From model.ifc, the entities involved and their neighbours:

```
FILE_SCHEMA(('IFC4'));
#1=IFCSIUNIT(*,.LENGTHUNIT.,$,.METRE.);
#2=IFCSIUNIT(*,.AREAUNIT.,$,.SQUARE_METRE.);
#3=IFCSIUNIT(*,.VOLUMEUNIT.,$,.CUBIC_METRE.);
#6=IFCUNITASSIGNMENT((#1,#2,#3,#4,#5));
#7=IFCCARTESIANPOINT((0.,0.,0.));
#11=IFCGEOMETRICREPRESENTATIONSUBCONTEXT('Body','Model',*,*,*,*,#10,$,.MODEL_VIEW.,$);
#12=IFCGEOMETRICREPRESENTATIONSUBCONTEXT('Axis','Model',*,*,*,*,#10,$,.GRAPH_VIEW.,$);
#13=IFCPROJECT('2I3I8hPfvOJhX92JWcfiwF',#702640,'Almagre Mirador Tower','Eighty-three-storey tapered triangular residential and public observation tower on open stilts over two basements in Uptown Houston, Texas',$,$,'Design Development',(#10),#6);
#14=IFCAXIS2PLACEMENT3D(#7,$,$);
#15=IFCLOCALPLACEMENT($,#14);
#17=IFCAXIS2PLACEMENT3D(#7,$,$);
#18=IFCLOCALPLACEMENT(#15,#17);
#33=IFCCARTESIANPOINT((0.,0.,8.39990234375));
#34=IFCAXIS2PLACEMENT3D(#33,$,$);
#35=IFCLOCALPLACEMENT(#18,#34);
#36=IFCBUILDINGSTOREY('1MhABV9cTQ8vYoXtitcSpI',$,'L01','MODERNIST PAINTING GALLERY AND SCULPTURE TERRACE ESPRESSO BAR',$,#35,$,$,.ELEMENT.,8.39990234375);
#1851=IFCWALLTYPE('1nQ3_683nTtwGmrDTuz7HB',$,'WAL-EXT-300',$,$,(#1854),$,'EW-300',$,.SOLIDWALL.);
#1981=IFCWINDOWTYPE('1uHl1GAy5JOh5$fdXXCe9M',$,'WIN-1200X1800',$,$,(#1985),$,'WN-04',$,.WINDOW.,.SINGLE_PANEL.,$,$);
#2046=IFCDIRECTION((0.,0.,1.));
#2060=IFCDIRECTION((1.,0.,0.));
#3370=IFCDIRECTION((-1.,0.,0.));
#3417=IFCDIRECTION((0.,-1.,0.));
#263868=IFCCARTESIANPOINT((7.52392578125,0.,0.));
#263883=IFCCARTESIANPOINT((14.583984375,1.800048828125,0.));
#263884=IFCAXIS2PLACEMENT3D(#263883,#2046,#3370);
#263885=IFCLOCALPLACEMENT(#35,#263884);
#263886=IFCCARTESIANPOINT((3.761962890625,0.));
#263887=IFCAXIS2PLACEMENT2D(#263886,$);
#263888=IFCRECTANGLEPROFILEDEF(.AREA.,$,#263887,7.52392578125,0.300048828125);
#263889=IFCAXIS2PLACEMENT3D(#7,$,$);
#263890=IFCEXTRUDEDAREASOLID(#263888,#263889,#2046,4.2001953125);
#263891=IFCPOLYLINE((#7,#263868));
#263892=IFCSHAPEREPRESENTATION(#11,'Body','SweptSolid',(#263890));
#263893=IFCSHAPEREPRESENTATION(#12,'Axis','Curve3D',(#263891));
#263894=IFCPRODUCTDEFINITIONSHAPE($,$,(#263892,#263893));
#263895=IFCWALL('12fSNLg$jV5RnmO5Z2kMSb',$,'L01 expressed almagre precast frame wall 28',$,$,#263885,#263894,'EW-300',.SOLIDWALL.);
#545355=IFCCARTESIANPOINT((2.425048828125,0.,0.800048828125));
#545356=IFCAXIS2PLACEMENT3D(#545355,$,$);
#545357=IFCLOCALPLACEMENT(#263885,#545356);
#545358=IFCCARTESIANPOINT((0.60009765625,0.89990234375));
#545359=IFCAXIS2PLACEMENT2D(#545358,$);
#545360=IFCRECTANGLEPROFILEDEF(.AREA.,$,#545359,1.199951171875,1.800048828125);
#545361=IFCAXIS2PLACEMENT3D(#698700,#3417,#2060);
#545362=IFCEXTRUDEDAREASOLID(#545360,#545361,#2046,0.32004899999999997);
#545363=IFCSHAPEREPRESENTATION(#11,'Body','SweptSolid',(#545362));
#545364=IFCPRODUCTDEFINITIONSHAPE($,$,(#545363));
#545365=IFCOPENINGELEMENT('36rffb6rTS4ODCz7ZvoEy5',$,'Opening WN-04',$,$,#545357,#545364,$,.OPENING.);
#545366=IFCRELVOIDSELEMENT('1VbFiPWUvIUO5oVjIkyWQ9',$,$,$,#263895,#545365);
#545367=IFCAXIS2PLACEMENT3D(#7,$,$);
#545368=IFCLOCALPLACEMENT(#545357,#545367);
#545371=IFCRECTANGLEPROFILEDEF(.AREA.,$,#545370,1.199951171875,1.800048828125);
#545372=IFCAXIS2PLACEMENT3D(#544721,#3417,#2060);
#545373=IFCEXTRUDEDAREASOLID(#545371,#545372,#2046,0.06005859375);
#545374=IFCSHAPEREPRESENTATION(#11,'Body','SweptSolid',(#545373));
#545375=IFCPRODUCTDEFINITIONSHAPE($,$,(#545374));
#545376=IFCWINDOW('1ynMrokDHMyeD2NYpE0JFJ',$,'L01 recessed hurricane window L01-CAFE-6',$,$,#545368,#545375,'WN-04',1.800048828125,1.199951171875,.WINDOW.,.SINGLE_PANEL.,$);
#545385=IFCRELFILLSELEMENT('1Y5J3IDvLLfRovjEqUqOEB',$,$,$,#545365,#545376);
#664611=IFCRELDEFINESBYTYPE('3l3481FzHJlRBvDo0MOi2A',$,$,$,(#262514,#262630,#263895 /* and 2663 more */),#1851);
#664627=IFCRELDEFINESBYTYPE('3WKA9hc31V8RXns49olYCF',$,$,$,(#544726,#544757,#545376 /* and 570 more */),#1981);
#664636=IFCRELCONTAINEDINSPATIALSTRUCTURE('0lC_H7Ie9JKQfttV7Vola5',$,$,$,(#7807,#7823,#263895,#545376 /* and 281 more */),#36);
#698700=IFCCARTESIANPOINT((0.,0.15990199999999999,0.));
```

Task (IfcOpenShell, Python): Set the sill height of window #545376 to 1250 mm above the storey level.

```python
import numpy as np
import ifcopenshell
import ifcopenshell.api.geometry
import ifcopenshell.geom
import ifcopenshell.util.element
import ifcopenshell.util.placement
import ifcopenshell.util.shape
import ifcopenshell.util.unit

model = ifcopenshell.open("model.ifc")
unit_scale = ifcopenshell.util.unit.calculate_unit_scale(model)

window = model.by_guid("1ynMrokDHMyeD2NYpE0JFJ")
opening = window.FillsVoids[0].RelatingOpeningElement
storey = ifcopenshell.util.element.get_container(window, ifc_class="IfcBuildingStorey")
level = ifcopenshell.util.placement.get_local_placement(storey.ObjectPlacement)[2, 3]

# The opening's origin need not be at the sill, so measure its lowest point.
shape = ifcopenshell.geom.create_shape(ifcopenshell.geom.settings(), opening)
bottom = ifcopenshell.util.shape.get_shape_bottom_elevation(shape, shape.geometry) / unit_scale
dz = level + 1.25 / unit_scale - bottom

shift = np.array([0.0, 0.0, dz])
# The window is placed relative to its opening, so it follows when the opening moves.
matrix = ifcopenshell.util.placement.get_local_placement(opening.ObjectPlacement)
matrix[:3, 3] += shift
ifcopenshell.api.geometry.edit_object_placement(
    model, product=opening, matrix=matrix, is_si=False, should_transform_children=True
)

print(f"moved by {dz * unit_scale:+.3f} m")

model.write("model_edited.ifc")
```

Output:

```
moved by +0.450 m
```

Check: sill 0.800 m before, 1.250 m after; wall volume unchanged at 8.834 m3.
